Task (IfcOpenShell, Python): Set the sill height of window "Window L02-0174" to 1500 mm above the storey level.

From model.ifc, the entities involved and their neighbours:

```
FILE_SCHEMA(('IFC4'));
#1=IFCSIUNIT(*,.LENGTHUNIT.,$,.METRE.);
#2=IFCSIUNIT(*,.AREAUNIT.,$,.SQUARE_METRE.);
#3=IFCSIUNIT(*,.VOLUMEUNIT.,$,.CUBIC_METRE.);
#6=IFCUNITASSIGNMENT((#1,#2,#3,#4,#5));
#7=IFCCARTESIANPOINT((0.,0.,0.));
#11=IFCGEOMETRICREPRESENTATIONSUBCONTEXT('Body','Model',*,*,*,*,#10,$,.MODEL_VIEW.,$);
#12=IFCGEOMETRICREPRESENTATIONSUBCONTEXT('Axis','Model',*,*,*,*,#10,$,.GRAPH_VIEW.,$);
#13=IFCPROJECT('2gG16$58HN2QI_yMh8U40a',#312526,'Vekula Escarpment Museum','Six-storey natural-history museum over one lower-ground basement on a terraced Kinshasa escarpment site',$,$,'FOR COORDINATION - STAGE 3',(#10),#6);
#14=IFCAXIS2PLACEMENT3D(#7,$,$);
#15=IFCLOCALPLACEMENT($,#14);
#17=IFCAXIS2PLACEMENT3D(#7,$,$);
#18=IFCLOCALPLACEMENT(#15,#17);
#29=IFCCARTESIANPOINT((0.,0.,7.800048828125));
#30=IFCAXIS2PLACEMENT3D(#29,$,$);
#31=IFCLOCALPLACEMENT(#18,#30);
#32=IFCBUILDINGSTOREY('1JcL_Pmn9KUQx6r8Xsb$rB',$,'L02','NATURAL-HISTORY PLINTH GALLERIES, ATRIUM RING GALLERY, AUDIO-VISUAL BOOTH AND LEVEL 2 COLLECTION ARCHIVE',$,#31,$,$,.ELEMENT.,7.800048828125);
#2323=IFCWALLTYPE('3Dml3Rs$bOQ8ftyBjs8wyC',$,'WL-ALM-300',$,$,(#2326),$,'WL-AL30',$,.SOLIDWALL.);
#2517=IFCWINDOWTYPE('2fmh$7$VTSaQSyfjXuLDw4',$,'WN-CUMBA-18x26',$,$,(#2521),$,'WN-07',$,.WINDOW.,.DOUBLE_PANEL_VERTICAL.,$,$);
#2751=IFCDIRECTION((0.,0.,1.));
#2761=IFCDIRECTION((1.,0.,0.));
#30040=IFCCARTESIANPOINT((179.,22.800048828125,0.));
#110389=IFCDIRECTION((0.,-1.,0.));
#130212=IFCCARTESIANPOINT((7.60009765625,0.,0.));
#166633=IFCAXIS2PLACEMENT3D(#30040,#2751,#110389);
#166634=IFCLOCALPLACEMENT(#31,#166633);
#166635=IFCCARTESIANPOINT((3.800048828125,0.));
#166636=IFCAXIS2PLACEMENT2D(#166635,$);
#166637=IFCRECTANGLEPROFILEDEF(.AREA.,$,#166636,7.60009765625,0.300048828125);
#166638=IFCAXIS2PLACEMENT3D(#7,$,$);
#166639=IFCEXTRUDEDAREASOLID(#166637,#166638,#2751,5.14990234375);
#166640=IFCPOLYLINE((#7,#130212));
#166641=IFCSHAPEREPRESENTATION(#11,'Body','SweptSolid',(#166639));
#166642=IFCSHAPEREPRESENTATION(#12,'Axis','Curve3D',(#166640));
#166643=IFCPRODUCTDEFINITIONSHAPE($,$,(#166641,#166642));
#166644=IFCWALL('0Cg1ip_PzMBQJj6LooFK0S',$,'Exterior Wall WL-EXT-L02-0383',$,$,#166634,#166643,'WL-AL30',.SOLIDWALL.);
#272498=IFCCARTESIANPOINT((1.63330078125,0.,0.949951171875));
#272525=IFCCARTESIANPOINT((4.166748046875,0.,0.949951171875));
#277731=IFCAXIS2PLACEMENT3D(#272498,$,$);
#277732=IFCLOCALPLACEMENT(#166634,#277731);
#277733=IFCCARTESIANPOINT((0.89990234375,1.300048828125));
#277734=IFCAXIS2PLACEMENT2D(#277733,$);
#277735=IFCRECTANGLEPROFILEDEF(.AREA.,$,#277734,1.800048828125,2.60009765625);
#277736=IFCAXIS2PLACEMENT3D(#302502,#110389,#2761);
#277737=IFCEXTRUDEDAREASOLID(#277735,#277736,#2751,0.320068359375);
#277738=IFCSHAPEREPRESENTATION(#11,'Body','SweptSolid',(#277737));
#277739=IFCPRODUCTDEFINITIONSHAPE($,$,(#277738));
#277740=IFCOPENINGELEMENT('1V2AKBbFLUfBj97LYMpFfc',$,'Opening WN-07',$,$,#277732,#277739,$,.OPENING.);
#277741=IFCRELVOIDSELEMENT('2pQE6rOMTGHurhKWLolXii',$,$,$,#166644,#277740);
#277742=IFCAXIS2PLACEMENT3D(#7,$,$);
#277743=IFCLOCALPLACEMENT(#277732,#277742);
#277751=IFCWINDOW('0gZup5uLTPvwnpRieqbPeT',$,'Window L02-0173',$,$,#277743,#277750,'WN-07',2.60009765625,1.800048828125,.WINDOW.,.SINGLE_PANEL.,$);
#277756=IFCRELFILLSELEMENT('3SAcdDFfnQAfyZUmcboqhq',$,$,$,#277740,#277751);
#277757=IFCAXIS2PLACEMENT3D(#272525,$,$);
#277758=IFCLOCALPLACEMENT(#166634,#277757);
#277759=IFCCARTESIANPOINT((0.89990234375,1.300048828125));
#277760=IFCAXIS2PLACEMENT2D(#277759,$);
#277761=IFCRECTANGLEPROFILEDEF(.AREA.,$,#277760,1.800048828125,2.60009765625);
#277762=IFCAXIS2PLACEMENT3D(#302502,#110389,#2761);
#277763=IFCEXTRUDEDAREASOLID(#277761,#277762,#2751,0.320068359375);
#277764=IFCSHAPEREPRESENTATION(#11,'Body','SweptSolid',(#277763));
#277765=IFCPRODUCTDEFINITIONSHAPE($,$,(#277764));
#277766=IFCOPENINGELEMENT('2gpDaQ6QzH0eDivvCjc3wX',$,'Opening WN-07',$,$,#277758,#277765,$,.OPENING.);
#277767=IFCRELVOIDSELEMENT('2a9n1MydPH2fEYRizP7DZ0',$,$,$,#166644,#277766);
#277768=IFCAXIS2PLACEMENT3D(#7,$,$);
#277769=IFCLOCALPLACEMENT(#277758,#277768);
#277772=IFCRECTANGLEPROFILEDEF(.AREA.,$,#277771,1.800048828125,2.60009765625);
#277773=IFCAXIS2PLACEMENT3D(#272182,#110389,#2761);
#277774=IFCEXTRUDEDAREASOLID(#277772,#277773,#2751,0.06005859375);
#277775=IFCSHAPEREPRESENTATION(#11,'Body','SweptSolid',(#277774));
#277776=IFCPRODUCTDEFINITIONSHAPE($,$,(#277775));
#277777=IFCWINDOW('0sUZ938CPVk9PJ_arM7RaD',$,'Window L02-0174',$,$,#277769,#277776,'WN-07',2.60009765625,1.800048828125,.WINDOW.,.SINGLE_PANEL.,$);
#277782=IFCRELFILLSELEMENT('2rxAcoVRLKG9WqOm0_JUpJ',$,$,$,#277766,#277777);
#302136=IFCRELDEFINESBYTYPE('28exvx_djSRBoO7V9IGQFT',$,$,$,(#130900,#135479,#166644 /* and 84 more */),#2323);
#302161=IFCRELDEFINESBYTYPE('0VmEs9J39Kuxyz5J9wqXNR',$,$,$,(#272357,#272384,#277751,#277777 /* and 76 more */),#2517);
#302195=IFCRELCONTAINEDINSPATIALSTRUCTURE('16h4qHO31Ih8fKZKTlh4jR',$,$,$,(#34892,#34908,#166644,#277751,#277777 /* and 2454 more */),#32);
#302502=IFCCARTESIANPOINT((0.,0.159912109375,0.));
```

```python
import numpy as np
import ifcopenshell
import ifcopenshell.api.geometry
import ifcopenshell.geom
import ifcopenshell.util.element
import ifcopenshell.util.placement
import ifcopenshell.util.shape
import ifcopenshell.util.unit

model = ifcopenshell.open("model.ifc")
unit_scale = ifcopenshell.util.unit.calculate_unit_scale(model)

window = model.by_guid("0sUZ938CPVk9PJ_arM7RaD")
opening = window.FillsVoids[0].RelatingOpeningElement
storey = ifcopenshell.util.element.get_container(window, ifc_class="IfcBuildingStorey")
level = ifcopenshell.util.placement.get_local_placement(storey.ObjectPlacement)[2, 3]

# The opening's origin need not be at the sill, so measure its lowest point.
shape = ifcopenshell.geom.create_shape(ifcopenshell.geom.settings(), opening)
bottom = ifcopenshell.util.shape.get_shape_bottom_elevation(shape, shape.geometry) / unit_scale
dz = level + 1.5 - bottom

shift = np.array([0.0, 0.0, dz])
# The window is placed relative to its opening, so it follows when the opening moves.
matrix = ifcopenshell.util.placement.get_local_placement(opening.ObjectPlacement)
matrix[:3, 3] += shift
ifcopenshell.api.geometry.edit_object_placement(
    model, product=opening, matrix=matrix, is_si=False, should_transform_children=True
)

print(f"moved by {dz * unit_scale:+.3f} m")

model.write("model_updated.ifc")
```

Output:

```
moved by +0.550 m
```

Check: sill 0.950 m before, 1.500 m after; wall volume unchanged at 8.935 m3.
